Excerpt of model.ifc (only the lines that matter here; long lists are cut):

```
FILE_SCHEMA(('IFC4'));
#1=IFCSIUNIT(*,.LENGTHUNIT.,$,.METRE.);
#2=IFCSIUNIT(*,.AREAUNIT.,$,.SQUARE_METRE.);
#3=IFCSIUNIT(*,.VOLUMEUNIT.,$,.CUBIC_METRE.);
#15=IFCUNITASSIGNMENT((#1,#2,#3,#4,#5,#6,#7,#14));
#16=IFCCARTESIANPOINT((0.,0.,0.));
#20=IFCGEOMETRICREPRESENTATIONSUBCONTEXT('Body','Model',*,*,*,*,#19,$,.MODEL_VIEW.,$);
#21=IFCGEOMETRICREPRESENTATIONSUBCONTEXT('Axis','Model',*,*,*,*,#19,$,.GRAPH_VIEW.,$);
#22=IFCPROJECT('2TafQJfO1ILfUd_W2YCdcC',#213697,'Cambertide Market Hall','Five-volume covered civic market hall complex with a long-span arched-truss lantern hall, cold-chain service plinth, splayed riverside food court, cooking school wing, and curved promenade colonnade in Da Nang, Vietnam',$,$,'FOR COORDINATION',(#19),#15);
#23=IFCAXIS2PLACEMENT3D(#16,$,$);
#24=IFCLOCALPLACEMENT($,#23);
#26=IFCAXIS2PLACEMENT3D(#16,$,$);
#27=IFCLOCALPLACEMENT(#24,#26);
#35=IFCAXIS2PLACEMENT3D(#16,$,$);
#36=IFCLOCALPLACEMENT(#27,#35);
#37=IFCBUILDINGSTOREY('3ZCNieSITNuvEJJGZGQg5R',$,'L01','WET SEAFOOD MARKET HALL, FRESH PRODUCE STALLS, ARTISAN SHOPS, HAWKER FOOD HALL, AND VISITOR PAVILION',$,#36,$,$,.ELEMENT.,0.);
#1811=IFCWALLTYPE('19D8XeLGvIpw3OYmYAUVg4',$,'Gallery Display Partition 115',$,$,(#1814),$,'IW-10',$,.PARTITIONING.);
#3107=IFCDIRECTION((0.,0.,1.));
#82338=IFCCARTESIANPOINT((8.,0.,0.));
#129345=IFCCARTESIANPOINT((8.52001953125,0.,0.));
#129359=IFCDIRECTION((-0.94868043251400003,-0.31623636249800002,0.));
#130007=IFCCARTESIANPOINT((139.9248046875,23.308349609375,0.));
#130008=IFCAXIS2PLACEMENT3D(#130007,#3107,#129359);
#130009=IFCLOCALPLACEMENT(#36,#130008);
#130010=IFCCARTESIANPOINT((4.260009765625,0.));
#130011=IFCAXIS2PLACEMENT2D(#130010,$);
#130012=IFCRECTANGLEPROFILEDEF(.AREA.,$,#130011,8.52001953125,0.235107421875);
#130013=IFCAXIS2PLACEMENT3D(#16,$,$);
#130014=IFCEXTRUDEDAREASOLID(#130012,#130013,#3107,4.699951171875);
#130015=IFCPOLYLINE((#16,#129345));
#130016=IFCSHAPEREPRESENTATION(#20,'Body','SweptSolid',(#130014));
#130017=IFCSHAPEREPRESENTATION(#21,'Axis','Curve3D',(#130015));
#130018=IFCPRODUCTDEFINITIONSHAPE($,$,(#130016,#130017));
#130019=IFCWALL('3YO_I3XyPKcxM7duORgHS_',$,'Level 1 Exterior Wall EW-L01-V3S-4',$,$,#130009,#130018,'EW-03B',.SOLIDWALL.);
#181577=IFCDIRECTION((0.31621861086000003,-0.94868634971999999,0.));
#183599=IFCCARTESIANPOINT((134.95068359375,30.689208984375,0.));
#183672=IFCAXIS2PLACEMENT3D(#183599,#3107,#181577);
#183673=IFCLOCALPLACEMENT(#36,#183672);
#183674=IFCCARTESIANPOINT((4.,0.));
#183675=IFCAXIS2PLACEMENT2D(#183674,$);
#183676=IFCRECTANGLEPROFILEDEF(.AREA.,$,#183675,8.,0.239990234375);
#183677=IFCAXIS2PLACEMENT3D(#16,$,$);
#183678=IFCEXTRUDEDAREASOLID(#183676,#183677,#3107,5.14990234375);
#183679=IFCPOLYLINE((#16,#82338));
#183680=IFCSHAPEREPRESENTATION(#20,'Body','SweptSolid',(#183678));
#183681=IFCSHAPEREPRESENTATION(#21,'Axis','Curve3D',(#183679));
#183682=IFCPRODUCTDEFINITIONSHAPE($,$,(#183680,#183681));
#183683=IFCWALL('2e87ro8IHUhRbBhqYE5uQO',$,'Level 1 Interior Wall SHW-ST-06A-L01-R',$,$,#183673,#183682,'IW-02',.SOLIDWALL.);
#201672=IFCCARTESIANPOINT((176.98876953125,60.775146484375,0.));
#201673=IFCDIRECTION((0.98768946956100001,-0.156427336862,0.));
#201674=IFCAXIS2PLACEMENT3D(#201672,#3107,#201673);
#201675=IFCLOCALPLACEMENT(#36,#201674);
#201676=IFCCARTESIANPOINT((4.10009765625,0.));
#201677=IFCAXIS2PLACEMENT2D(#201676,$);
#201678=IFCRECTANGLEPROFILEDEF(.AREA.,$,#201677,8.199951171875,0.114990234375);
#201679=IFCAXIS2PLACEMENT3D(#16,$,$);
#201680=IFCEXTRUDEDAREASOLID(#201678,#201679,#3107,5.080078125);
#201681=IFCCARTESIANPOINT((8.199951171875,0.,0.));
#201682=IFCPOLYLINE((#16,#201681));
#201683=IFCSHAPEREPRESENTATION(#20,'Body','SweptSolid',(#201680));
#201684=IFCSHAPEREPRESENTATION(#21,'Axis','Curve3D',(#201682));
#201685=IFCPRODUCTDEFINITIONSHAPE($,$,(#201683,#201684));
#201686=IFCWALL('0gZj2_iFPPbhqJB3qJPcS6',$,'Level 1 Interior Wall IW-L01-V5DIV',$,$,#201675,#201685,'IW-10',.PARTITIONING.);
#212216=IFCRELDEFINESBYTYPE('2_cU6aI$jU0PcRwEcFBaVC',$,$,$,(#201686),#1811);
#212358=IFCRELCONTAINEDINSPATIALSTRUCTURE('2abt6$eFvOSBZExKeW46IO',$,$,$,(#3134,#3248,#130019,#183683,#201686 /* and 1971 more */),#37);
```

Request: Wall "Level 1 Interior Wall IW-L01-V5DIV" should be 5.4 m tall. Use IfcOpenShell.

```python
import ifcopenshell
import ifcopenshell.geom
import ifcopenshell.util.representation
import ifcopenshell.util.shape

model = ifcopenshell.open("model.ifc")
settings = ifcopenshell.geom.settings()


def volume(element):
    """Net volume in cubic metres, openings subtracted."""
    shape = ifcopenshell.geom.create_shape(settings, element)
    return ifcopenshell.util.shape.get_volume(shape.geometry)


wall = model.by_id(201686)
before = volume(wall)

body = ifcopenshell.util.representation.get_representation(wall, "Model", "Body")
solid = body.Items[0]
old_height = solid.Depth
solid.Depth = 5.4
after = volume(wall)

print(f"height {old_height:g} -> {solid.Depth:g}, volume {before:.3f} -> {after:.3f} m3")

model.write("model-out.ifc")
```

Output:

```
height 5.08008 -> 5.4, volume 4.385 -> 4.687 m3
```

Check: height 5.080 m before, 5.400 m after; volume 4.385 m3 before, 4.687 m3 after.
